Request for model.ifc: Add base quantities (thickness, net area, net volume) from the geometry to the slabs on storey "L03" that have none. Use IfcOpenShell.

First a look at what the model holds.

```python
import ifcopenshell
import ifcopenshell.util.element
import ifcopenshell.util.unit

model = ifcopenshell.open("model.ifc")
print(model.schema)
for unit_type in ("LENGTHUNIT", "AREAUNIT", "VOLUMEUNIT"):
    print(unit_type, ifcopenshell.util.unit.calculate_unit_scale(model, unit_type))
storey = next(s for s in model.by_type("IfcBuildingStorey") if s.Name == "L03")
slabs = [e for e in ifcopenshell.util.element.get_decomposition(storey) if e.is_a("IfcSlab")]
for e in sorted(slabs, key=lambda e: e.id()):
    print(e.id(), e.is_a(), e.Name, list(ifcopenshell.util.element.get_psets(e, qtos_only=True)), sep=" | ")
```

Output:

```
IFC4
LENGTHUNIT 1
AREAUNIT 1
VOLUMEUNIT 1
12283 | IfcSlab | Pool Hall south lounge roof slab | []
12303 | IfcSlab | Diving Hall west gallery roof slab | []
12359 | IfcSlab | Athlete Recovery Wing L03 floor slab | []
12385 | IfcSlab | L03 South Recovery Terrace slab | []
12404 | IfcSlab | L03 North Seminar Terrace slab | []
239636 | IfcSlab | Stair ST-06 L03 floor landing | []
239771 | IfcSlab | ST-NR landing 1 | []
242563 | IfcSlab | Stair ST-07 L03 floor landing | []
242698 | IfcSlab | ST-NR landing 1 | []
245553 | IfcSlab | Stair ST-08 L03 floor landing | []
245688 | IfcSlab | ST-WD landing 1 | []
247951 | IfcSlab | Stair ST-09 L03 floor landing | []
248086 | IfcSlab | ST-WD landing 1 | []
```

```python
import ifcopenshell
import ifcopenshell.api.pset
import ifcopenshell.geom
import ifcopenshell.util.element
import ifcopenshell.util.shape
import ifcopenshell.util.unit

model = ifcopenshell.open("model.ifc")
unit_scale = ifcopenshell.util.unit.calculate_unit_scale(model)
area_scale = ifcopenshell.util.unit.calculate_unit_scale(model, "AREAUNIT")
volume_scale = ifcopenshell.util.unit.calculate_unit_scale(model, "VOLUMEUNIT")
settings = ifcopenshell.geom.settings()

storey = next(s for s in model.by_type("IfcBuildingStorey") if s.Name == "L03")
slabs = [e for e in ifcopenshell.util.element.get_decomposition(storey) if e.is_a("IfcSlab")]

for e in sorted(slabs, key=lambda e: e.id()):
    if ifcopenshell.util.element.get_psets(e, qtos_only=True, should_inherit=False):
        continue
    # Geometry comes back in metres, in the element's own axes.
    shape = ifcopenshell.geom.create_shape(settings, e)
    values = {
        "Width": ifcopenshell.util.shape.get_z(shape.geometry) / unit_scale,
        "NetArea": ifcopenshell.util.shape.get_footprint_area(shape.geometry) / area_scale,
        "NetVolume": ifcopenshell.util.shape.get_volume(shape.geometry) / volume_scale,
    }
    qto = ifcopenshell.api.pset.add_qto(model, product=e, name="Qto_SlabBaseQuantities")
    ifcopenshell.api.pset.edit_qto(model, qto=qto, properties=values)
    print(e.id(), {k: round(v, 3) for k, v in values.items()})

model.write("model_edited.ifc")
```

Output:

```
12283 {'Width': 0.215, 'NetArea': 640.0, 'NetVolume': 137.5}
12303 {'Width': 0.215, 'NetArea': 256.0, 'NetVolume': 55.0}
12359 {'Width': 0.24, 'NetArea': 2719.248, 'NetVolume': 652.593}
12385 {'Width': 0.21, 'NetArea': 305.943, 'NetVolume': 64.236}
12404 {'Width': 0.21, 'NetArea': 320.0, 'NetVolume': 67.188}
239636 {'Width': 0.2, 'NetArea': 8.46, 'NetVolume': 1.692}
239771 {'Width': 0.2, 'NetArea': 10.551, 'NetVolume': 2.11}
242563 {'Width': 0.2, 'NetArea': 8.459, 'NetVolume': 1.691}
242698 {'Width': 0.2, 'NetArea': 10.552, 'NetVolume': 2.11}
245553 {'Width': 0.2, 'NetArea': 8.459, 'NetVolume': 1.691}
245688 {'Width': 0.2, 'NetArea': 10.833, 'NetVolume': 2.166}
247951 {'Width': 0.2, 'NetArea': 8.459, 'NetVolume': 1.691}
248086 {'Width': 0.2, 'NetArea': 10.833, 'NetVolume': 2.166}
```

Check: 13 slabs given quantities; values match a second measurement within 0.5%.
